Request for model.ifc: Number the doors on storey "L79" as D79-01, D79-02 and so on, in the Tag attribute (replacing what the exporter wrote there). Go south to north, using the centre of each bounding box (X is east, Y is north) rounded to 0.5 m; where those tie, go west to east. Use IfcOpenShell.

First a look at what the model holds.

```python
import ifcopenshell
import ifcopenshell.util.element
import ifcopenshell.util.placement

model = ifcopenshell.open("model.ifc")
print(model.schema)
storey = next(s for s in model.by_type("IfcBuildingStorey") if s.Name == "L79")
doors = [e for e in ifcopenshell.util.element.get_decomposition(storey) if e.is_a("IfcDoor")]
for e in sorted(doors, key=lambda e: e.id()):
    origin = ifcopenshell.util.placement.get_local_placement(e.ObjectPlacement)[:3, 3]
    print(e.id(), e.Tag, e.Name, origin.round(2) + 0.0, sep=" | ")
```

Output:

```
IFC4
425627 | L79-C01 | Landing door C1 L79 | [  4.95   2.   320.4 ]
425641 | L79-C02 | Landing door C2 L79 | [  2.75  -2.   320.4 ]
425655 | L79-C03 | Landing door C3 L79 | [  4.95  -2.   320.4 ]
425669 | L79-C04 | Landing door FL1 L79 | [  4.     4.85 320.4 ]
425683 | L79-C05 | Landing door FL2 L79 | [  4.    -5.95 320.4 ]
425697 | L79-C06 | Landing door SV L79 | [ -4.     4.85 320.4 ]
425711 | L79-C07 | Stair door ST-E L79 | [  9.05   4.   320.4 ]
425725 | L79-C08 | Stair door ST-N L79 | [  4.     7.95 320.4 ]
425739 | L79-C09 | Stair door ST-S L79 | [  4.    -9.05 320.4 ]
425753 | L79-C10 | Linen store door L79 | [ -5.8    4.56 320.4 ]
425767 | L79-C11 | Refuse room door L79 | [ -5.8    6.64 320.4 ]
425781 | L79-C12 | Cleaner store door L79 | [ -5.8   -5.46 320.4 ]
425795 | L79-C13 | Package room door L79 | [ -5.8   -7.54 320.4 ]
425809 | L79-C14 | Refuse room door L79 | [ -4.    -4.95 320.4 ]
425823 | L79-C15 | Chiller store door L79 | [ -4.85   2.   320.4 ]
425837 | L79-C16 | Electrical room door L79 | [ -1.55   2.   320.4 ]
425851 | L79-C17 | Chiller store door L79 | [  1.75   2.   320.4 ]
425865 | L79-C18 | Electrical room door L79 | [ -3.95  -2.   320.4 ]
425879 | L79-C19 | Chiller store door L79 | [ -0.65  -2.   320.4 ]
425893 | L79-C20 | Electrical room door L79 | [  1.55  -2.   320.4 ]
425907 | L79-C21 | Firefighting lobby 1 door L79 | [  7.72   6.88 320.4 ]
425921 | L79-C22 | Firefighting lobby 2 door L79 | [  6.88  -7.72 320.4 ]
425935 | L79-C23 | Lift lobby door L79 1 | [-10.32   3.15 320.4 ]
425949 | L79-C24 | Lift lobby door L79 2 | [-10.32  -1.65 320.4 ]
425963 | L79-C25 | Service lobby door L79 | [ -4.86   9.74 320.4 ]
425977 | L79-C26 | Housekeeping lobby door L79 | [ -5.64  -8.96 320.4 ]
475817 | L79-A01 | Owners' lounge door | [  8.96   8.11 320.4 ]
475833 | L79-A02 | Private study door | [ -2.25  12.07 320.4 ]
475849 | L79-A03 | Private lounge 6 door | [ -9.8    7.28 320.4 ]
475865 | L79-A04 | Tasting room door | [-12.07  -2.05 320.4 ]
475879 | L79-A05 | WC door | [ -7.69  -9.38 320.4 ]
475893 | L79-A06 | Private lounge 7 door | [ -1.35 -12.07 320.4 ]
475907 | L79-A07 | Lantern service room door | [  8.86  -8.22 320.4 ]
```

```python
import ifcopenshell
import ifcopenshell.geom
import ifcopenshell.util.element
import ifcopenshell.util.shape

model = ifcopenshell.open("model.ifc")
settings = ifcopenshell.geom.settings()
settings.set("use-world-coords", True)


def centre(element):
    shape = ifcopenshell.geom.create_shape(settings, element)
    return ifcopenshell.util.shape.get_bbox_centroid(shape.geometry)


storey = next(s for s in model.by_type("IfcBuildingStorey") if s.Name == "L79")
doors = [e for e in ifcopenshell.util.element.get_decomposition(storey) if e.is_a("IfcDoor")]

# Insertion points can sit at a corner or the storey origin, so sort by the geometry (in metres).
centres = {e: centre(e) for e in doors}
doors.sort(key=lambda e: (round(centres[e][1] / 0.5), centres[e][0]))

for i, e in enumerate(doors, start=1):
    number = f"D79-{i:02d}"
    e.Tag = number
    print(e.id(), number)

model.write("model_updated.ifc")
```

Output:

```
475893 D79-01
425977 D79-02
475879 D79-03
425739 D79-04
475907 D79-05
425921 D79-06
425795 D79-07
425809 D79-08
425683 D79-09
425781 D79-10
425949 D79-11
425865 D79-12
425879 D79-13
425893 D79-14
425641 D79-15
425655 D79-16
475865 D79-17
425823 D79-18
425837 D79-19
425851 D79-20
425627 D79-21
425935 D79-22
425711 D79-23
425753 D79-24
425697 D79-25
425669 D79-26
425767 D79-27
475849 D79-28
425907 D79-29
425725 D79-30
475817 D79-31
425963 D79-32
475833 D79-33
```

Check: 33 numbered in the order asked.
